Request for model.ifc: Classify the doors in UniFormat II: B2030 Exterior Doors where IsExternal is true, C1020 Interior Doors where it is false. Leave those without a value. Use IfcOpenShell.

First a look at what the model holds.

```python
import ifcopenshell
import ifcopenshell.util.element

model = ifcopenshell.open("model.ifc")
print(model.schema)
print("classifications:", [c.Name for c in model.by_type("IfcClassification")])
values = [ifcopenshell.util.element.get_pset(e, "Pset_DoorCommon", "IsExternal") for e in model.by_type("IfcDoor")]
for value in (True, False, None):
    print("IsExternal", value, values.count(value))
```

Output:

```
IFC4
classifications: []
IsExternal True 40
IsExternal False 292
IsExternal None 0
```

```python
import ifcopenshell
import ifcopenshell.api.classification
import ifcopenshell.util.element

model = ifcopenshell.open("model.ifc")

system = ifcopenshell.api.classification.add_classification(model, classification="UniFormat II")

doors = model.by_type("IfcDoor")
external = {e: ifcopenshell.util.element.get_pset(e, "Pset_DoorCommon", "IsExternal") for e in doors}
for flag, code, name in ((True, "B2030", "Exterior Doors"), (False, "C1020", "Interior Doors")):
    products = [e for e in doors if external[e] is flag]
    ifcopenshell.api.classification.add_reference(
        model, products=products, classification=system, identification=code, name=name
    )
    print(code, len(products))

model.write("model_v2.ifc")
```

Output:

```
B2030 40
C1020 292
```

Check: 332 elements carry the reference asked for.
